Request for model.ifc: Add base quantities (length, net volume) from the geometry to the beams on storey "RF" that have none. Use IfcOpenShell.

First a look at what the model holds.

```python
import ifcopenshell
import ifcopenshell.util.element
import ifcopenshell.util.unit

model = ifcopenshell.open("model.ifc")
print(model.schema)
for unit_type in ("LENGTHUNIT", "AREAUNIT", "VOLUMEUNIT"):
    print(unit_type, ifcopenshell.util.unit.calculate_unit_scale(model, unit_type))
storey = next(s for s in model.by_type("IfcBuildingStorey") if s.Name == "RF")
beams = [e for e in ifcopenshell.util.element.get_decomposition(storey) if e.is_a("IfcBeam")]
for e in sorted(beams, key=lambda e: e.id()):
    print(e.id(), e.is_a(), e.Name, list(ifcopenshell.util.element.get_psets(e, qtos_only=True)), sep=" | ")
```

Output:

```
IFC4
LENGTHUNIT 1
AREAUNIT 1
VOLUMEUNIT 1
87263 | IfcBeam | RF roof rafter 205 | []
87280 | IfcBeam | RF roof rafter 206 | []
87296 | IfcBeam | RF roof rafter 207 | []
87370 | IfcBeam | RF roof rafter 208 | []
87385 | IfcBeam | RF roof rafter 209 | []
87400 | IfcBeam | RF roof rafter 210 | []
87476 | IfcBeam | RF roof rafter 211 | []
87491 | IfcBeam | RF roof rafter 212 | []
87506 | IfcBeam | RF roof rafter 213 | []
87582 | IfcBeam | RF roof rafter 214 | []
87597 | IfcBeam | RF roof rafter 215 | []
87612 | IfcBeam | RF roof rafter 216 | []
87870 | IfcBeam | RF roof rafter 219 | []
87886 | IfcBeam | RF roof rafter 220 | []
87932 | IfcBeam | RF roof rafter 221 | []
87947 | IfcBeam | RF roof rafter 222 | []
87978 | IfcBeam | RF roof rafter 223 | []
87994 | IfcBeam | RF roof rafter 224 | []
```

```python
import ifcopenshell
import ifcopenshell.api.pset
import ifcopenshell.geom
import ifcopenshell.util.element
import ifcopenshell.util.shape
import ifcopenshell.util.unit

model = ifcopenshell.open("model.ifc")
unit_scale = ifcopenshell.util.unit.calculate_unit_scale(model)
volume_scale = ifcopenshell.util.unit.calculate_unit_scale(model, "VOLUMEUNIT")
settings = ifcopenshell.geom.settings()

storey = next(s for s in model.by_type("IfcBuildingStorey") if s.Name == "RF")
beams = [e for e in ifcopenshell.util.element.get_decomposition(storey) if e.is_a("IfcBeam")]

for e in sorted(beams, key=lambda e: e.id()):
    if ifcopenshell.util.element.get_psets(e, qtos_only=True, should_inherit=False):
        continue
    # Geometry comes back in metres, in the element's own axes.
    shape = ifcopenshell.geom.create_shape(settings, e)
    values = {
        "Length": ifcopenshell.util.shape.get_max_xyz(shape.geometry) / unit_scale,
        "NetVolume": ifcopenshell.util.shape.get_volume(shape.geometry) / volume_scale,
    }
    qto = ifcopenshell.api.pset.add_qto(model, product=e, name="Qto_BeamBaseQuantities")
    ifcopenshell.api.pset.edit_qto(model, qto=qto, properties=values)
    print(e.id(), {k: round(v, 3) for k, v in values.items()})

model.write("model_updated.ifc")
```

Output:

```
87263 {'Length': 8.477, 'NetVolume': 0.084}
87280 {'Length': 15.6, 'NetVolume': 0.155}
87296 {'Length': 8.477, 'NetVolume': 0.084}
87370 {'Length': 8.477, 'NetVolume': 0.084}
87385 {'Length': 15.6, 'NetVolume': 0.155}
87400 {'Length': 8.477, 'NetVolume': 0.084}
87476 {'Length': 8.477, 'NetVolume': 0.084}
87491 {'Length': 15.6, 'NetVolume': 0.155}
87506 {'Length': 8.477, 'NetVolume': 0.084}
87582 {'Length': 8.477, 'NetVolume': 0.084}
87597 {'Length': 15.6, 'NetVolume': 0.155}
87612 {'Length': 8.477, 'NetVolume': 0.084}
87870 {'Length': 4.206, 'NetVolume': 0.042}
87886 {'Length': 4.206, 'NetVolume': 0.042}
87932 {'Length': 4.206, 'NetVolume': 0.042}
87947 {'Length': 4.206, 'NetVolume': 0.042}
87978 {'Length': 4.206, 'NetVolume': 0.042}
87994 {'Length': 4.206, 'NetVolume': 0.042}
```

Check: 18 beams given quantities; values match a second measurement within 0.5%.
